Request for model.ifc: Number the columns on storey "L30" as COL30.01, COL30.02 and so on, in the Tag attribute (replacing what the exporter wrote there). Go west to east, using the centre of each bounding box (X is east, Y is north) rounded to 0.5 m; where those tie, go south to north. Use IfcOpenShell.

First a look at what the model holds.

```python
import ifcopenshell
import ifcopenshell.util.element
import ifcopenshell.util.placement

model = ifcopenshell.open("model.ifc")
print(model.schema)
storey = next(s for s in model.by_type("IfcBuildingStorey") if s.Name == "L30")
columns = [e for e in ifcopenshell.util.element.get_decomposition(storey) if e.is_a("IfcColumn")]
for e in sorted(columns, key=lambda e: e.id()):
    origin = ifcopenshell.util.placement.get_local_placement(e.ObjectPlacement)[:3, 3]
    print(e.id(), e.Tag, e.Name, origin.round(2) + 0.0, sep=" | ")
```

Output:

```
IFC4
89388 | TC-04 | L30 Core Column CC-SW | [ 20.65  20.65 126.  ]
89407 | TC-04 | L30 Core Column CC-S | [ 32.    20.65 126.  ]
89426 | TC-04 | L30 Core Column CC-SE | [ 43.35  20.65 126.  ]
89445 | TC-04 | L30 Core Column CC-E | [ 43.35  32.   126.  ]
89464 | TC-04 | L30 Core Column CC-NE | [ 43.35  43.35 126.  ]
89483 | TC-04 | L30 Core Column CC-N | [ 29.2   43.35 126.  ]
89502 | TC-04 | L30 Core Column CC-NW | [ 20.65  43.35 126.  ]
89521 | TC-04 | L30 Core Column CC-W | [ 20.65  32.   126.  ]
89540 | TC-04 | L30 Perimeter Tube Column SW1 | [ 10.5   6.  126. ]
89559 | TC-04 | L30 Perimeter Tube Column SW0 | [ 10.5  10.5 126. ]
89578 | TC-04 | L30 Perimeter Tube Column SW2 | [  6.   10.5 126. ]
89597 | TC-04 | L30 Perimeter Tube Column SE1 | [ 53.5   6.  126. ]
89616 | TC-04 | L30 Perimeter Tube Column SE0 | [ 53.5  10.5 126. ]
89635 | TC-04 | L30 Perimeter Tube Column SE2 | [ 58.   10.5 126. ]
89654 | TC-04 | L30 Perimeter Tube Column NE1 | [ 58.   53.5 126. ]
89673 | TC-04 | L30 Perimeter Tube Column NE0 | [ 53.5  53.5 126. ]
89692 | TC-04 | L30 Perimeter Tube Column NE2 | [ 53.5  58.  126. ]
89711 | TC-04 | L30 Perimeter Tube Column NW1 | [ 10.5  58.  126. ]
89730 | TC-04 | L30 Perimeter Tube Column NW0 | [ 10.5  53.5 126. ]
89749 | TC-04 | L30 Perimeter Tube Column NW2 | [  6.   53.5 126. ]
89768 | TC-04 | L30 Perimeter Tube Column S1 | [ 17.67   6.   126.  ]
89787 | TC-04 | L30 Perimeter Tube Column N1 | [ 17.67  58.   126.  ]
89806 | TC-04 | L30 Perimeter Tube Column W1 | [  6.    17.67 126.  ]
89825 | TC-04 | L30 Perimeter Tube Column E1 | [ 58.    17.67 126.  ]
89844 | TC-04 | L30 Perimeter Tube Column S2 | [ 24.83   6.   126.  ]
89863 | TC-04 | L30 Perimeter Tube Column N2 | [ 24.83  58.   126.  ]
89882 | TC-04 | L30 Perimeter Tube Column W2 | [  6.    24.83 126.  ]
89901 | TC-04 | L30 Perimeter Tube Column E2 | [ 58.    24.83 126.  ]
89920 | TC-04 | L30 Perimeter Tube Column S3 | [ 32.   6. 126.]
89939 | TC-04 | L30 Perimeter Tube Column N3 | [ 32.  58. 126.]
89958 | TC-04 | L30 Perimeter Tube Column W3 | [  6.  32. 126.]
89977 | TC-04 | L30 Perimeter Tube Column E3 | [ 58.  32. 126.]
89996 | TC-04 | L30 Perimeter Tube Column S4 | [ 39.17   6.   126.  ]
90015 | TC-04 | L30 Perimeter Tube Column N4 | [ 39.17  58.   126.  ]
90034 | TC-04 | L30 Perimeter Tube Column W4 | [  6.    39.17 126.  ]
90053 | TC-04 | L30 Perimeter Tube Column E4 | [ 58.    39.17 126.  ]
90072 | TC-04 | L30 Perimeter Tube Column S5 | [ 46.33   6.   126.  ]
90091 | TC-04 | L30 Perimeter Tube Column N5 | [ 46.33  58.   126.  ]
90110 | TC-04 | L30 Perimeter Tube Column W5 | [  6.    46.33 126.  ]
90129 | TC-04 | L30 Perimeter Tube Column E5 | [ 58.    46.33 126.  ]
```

```python
import ifcopenshell
import ifcopenshell.geom
import ifcopenshell.util.element
import ifcopenshell.util.shape

model = ifcopenshell.open("model.ifc")
settings = ifcopenshell.geom.settings()
settings.set("use-world-coords", True)


def centre(element):
    shape = ifcopenshell.geom.create_shape(settings, element)
    return ifcopenshell.util.shape.get_bbox_centroid(shape.geometry)


storey = next(s for s in model.by_type("IfcBuildingStorey") if s.Name == "L30")
columns = [e for e in ifcopenshell.util.element.get_decomposition(storey) if e.is_a("IfcColumn")]

# Insertion points can sit at a corner or the storey origin, so sort by the geometry (in metres).
centres = {e: centre(e) for e in columns}
columns.sort(key=lambda e: (round(centres[e][0] / 0.5), centres[e][1]))

for i, e in enumerate(columns, start=1):
    number = f"COL30.{i:02d}"
    e.Tag = number
    print(e.id(), number)

model.write("model-out.ifc")
```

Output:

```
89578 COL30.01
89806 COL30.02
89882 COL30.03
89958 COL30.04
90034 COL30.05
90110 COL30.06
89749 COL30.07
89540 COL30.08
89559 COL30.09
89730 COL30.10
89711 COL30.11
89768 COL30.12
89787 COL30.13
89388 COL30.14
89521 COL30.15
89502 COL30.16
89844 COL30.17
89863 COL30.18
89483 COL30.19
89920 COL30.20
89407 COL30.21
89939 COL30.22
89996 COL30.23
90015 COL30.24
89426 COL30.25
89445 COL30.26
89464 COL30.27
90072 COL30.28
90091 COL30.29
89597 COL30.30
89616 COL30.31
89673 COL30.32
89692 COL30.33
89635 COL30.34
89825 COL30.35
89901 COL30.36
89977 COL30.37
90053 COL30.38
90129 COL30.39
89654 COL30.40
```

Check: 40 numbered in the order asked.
